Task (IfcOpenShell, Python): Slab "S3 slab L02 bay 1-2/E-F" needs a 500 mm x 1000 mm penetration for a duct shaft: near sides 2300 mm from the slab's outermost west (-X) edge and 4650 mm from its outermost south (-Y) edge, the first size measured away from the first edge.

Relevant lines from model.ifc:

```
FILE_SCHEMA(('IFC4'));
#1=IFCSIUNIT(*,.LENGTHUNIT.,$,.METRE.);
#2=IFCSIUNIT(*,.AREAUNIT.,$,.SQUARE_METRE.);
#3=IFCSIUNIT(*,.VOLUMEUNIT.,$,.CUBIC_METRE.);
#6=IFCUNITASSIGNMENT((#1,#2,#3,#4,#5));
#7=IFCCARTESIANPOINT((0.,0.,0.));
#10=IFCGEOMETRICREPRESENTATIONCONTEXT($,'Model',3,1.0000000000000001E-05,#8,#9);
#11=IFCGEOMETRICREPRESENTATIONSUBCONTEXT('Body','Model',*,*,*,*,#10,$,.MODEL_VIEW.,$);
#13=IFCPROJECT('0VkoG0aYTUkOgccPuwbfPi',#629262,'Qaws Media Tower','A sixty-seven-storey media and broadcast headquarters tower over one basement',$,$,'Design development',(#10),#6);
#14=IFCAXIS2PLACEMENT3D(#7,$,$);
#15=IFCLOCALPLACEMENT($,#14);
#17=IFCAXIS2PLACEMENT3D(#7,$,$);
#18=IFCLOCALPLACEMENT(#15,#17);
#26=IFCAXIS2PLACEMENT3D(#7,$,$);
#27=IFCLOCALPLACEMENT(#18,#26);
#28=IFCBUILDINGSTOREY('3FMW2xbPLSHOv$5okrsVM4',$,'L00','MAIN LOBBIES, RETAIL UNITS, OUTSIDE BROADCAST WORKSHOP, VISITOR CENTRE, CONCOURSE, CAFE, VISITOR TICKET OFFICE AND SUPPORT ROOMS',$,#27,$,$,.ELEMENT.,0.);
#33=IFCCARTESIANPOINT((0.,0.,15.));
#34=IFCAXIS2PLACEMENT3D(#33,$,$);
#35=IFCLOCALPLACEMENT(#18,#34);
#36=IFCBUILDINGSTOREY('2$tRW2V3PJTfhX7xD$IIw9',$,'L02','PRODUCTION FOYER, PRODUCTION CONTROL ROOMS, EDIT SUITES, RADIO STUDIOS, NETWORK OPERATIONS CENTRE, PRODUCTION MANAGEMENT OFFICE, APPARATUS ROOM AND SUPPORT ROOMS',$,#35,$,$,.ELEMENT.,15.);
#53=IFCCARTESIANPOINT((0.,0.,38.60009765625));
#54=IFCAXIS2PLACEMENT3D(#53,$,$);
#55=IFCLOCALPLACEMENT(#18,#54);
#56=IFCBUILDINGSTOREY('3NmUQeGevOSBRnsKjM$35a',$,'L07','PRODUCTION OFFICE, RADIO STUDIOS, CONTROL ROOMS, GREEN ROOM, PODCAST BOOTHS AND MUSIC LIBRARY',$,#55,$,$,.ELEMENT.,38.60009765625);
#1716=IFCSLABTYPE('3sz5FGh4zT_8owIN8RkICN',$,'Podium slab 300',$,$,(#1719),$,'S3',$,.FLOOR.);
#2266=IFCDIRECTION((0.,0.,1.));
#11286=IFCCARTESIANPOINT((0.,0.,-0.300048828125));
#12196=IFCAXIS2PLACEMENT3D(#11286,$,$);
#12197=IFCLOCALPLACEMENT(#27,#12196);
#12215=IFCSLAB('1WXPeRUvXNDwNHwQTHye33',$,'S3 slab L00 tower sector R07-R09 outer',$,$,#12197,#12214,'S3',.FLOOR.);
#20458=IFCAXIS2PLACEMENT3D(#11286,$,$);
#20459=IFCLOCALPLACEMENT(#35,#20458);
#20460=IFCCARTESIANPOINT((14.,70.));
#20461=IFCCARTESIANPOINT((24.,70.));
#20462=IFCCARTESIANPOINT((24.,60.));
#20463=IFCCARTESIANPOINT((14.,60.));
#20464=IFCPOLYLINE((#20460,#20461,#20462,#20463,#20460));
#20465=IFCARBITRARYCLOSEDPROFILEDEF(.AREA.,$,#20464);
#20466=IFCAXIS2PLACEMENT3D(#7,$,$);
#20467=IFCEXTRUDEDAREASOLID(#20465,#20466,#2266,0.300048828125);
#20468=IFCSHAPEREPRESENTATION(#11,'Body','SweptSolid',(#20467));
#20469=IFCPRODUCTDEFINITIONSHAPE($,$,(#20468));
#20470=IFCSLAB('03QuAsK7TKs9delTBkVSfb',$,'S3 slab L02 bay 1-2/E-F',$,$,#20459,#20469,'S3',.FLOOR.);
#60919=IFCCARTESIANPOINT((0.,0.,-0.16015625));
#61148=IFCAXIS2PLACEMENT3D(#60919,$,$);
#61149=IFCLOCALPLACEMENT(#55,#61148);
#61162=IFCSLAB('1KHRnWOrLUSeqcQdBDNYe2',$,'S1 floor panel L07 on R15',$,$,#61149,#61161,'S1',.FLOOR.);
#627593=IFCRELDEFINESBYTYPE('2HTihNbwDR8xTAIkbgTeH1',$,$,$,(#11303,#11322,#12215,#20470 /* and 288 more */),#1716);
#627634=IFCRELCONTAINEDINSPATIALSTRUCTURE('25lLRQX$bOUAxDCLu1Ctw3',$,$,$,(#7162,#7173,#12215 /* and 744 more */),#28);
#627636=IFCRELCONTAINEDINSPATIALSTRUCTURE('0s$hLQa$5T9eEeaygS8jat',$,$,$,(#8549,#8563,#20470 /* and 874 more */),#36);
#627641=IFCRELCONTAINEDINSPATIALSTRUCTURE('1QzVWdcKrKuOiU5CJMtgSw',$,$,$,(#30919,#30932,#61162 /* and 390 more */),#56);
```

```python
import numpy as np
import ifcopenshell
import ifcopenshell.api.feature
import ifcopenshell.api.geometry
import ifcopenshell.api.root
import ifcopenshell.geom
import ifcopenshell.util.placement
import ifcopenshell.util.representation
import ifcopenshell.util.shape
import ifcopenshell.util.unit

model = ifcopenshell.open("model.ifc")
unit_scale = ifcopenshell.util.unit.calculate_unit_scale(model)
settings = ifcopenshell.geom.settings()


def volume(element):
    """Net volume in cubic metres, openings subtracted."""
    shape = ifcopenshell.geom.create_shape(settings, element)
    return ifcopenshell.util.shape.get_volume(shape.geometry)


slab = model.by_guid("03QuAsK7TKs9delTBkVSfb")
before = volume(slab)

# Extent in the slab's own axes, in metres. The edges named are its -X and -Y sides.
slab_shape = ifcopenshell.geom.create_shape(settings, slab)
vertices = ifcopenshell.util.shape.get_vertices(slab_shape.geometry)
x_min, y_min, bottom = vertices.min(axis=0)
top = vertices[:, 2].max()

opening = ifcopenshell.api.root.create_entity(model, ifc_class="IfcOpeningElement", name="Duct shaft opening", predefined_type="OPENING")
context = ifcopenshell.util.representation.get_context(model, "Model", "Body", "MODEL_VIEW")
width, depth = 0.5, 1
outline = [(0.0, 0.0), (width, 0.0), (width, depth), (0.0, depth), (0.0, 0.0)]
# Overshoot both faces by 50 mm so the cut is clean.
shape = ifcopenshell.api.geometry.add_slab_representation(
    model, context=context, depth=top - bottom + 0.1, polyline=outline
)
ifcopenshell.api.geometry.assign_representation(model, product=opening, representation=shape)

matrix = ifcopenshell.util.placement.get_local_placement(slab.ObjectPlacement)
matrix[:, 3] = matrix @ np.append(np.array([x_min + 2.3, y_min + 4.65, bottom - 0.05]) / unit_scale, 1.0)
ifcopenshell.api.geometry.edit_object_placement(model, product=opening, matrix=matrix, is_si=False)
ifcopenshell.api.feature.add_feature(model, feature=opening, element=slab)

after = volume(slab)

print(f"slab volume {before:.3f} -> {after:.3f} m3")

model.write("model_rev.ifc")
```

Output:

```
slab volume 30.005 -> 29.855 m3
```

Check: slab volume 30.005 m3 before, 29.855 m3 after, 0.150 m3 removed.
